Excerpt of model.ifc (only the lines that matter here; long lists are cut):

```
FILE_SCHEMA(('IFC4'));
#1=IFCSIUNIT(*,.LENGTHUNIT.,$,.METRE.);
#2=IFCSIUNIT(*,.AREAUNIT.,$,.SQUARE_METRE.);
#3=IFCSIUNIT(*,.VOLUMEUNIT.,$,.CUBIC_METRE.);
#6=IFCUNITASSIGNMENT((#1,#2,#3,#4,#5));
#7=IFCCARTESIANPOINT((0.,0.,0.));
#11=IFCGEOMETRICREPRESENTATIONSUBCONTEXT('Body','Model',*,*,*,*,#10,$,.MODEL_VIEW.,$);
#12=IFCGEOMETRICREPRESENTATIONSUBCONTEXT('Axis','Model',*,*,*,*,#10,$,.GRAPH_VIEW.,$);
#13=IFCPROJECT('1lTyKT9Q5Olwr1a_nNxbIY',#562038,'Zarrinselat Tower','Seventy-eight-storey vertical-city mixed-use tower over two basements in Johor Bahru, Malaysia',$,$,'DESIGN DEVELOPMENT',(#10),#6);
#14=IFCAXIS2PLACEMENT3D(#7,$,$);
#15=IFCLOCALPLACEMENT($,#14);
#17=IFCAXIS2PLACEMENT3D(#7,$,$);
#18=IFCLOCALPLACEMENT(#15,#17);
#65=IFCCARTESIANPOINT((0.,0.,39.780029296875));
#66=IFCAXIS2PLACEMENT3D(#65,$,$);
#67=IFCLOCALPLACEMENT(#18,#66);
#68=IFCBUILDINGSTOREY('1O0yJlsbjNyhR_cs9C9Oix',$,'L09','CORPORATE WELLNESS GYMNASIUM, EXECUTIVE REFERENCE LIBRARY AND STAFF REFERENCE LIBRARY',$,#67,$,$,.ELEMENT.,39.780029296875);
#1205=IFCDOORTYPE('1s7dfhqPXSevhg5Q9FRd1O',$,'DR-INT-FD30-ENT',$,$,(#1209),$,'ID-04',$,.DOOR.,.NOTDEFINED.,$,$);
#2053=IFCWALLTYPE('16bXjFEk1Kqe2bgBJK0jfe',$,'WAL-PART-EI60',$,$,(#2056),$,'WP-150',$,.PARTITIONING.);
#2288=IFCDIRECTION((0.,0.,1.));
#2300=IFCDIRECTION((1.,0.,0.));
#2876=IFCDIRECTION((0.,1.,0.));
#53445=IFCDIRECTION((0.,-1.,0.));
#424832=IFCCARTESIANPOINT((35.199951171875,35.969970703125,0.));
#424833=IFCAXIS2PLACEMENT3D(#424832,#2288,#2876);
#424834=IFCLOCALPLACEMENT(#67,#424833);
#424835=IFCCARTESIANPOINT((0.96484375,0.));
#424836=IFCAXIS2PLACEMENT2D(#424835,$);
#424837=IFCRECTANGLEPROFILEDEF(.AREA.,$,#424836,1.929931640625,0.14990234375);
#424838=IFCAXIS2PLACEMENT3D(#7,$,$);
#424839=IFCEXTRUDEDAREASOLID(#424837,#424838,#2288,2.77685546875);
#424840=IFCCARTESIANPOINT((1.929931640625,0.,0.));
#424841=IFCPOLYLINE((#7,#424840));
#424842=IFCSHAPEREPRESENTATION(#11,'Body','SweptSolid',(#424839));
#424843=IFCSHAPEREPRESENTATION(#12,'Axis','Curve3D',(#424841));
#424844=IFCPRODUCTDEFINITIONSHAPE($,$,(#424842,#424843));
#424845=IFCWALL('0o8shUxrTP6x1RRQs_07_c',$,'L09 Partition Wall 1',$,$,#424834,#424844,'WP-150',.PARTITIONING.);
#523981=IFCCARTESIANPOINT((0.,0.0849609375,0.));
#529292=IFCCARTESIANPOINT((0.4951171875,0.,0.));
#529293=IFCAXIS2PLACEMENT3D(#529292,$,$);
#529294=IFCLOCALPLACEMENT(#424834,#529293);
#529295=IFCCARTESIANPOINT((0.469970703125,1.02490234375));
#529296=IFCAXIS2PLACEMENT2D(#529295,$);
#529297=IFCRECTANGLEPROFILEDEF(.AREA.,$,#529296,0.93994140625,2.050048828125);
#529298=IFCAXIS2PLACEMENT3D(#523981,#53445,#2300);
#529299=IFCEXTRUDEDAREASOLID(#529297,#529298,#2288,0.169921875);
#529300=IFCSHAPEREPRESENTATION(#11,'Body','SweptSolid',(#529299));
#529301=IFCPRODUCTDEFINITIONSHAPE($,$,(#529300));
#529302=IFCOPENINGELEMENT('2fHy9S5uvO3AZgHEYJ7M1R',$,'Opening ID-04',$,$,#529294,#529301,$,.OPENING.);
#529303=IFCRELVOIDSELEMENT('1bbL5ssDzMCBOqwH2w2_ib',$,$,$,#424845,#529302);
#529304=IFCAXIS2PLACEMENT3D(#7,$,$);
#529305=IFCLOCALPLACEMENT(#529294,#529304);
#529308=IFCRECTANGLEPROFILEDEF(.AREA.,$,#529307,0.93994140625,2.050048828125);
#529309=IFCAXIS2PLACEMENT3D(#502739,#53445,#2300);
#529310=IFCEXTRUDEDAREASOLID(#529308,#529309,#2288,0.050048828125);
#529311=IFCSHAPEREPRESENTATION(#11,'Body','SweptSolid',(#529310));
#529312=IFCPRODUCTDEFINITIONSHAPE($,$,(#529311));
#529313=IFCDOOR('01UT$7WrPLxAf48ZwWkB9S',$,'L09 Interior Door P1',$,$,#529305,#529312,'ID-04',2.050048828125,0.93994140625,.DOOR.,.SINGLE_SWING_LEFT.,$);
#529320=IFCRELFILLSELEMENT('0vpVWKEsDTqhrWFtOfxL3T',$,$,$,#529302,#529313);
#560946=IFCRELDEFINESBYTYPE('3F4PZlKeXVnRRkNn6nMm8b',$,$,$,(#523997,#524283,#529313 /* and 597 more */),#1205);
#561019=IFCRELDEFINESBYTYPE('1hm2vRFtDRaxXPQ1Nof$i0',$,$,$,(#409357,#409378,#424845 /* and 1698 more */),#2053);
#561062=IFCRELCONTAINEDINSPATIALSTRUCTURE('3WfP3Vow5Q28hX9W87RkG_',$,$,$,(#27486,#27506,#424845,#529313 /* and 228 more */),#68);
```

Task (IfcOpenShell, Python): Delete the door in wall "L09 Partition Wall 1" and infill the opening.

```python
import ifcopenshell
import ifcopenshell.api.feature
import ifcopenshell.api.root
import ifcopenshell.geom
import ifcopenshell.util.shape

model = ifcopenshell.open("model.ifc")
settings = ifcopenshell.geom.settings()


def volume(element):
    """Net volume in cubic metres, openings subtracted."""
    shape = ifcopenshell.geom.create_shape(settings, element)
    return ifcopenshell.util.shape.get_volume(shape.geometry)


door = model.by_guid("01UT$7WrPLxAf48ZwWkB9S")
opening = door.FillsVoids[0].RelatingOpeningElement
wall = opening.VoidsElements[0].RelatingBuildingElement
before = volume(wall)

ifcopenshell.api.root.remove_product(model, product=door)
ifcopenshell.api.feature.remove_feature(model, feature=opening)

after = volume(wall)

print(f"wall volume {before:.3f} -> {after:.3f} m3")

model.write("model_edited.ifc")
```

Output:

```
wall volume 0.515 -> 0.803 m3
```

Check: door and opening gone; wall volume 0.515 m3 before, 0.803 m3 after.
